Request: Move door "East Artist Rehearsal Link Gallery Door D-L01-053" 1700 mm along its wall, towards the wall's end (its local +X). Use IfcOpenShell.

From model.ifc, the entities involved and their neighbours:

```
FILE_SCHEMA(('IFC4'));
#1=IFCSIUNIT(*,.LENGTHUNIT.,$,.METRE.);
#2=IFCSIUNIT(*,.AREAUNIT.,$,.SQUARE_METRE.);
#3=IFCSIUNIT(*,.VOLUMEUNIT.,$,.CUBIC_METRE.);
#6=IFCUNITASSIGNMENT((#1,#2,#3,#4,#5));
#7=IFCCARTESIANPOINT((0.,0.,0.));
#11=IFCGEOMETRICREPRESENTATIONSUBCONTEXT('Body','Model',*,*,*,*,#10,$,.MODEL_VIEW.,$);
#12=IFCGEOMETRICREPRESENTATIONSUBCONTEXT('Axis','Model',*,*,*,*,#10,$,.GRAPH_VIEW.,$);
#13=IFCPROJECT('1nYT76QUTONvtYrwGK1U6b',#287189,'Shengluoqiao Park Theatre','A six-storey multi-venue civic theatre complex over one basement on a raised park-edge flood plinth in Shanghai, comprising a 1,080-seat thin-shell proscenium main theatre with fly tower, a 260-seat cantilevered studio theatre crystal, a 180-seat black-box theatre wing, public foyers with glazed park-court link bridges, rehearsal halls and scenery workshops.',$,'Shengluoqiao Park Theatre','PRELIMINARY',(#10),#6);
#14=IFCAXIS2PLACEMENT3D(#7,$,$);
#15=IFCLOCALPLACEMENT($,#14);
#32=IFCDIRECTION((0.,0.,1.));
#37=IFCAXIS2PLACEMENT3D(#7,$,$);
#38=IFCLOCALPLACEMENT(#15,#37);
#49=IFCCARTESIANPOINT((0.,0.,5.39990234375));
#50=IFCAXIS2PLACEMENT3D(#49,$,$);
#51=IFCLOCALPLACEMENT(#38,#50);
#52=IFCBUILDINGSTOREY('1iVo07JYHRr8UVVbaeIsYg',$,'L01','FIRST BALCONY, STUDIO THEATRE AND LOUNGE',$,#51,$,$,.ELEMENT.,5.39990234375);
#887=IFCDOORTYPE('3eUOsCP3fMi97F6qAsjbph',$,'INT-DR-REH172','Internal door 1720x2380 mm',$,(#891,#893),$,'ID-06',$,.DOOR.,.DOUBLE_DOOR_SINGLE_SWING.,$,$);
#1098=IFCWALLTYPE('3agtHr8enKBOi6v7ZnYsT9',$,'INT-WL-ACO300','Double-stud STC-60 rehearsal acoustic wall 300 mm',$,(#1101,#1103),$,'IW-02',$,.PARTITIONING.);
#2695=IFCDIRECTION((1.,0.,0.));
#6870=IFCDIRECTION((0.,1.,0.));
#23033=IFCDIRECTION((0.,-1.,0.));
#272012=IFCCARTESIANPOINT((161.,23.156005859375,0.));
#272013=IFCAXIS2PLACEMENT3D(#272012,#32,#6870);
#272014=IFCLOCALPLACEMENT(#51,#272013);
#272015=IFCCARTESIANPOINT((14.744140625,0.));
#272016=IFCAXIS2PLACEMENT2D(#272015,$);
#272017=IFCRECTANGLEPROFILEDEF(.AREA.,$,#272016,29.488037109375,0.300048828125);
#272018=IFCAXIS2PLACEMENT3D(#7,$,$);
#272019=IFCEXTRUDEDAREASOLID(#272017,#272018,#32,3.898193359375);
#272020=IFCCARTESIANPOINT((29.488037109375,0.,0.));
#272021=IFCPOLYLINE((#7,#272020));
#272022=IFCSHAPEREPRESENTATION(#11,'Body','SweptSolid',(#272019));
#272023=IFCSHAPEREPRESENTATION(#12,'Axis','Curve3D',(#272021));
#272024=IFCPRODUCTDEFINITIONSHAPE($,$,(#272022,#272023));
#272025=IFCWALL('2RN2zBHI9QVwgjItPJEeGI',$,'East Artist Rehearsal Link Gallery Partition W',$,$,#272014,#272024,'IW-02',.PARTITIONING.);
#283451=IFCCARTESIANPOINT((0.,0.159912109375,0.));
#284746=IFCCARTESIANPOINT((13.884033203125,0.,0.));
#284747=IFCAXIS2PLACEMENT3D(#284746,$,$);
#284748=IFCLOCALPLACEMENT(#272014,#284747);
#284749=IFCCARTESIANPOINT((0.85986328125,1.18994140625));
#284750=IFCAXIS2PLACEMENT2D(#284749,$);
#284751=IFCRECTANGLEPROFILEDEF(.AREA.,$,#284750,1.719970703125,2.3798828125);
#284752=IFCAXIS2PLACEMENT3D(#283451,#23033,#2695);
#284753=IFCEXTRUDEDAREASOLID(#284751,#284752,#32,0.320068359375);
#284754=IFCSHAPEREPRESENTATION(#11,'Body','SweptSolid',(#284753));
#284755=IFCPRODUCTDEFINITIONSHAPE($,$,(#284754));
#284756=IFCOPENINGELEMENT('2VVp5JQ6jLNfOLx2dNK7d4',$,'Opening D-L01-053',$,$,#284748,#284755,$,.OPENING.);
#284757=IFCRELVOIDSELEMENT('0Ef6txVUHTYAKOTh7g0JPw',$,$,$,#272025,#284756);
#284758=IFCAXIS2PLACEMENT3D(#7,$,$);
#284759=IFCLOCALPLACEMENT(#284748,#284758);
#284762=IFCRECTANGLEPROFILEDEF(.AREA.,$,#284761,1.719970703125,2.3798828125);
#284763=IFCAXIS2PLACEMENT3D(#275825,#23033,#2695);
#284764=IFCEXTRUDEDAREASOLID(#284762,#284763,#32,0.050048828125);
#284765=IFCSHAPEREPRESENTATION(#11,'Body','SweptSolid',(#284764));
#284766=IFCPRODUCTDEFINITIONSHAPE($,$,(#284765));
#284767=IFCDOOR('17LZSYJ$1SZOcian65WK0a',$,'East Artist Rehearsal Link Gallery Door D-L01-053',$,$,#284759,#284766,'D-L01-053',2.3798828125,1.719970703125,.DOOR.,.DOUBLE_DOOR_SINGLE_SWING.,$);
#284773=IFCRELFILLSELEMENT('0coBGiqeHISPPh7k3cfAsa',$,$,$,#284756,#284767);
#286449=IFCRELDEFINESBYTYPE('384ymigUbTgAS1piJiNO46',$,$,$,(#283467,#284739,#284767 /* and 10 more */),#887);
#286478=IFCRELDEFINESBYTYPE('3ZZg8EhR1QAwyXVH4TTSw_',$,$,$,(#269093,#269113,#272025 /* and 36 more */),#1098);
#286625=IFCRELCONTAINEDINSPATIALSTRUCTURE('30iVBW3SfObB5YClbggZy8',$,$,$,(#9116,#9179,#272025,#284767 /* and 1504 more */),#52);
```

```python
import ifcopenshell
import ifcopenshell.api.geometry
import ifcopenshell.util.placement

model = ifcopenshell.open("model.ifc")

door = model.by_id(284767)
opening = door.FillsVoids[0].RelatingOpeningElement
wall = opening.VoidsElements[0].RelatingBuildingElement

wall_matrix = ifcopenshell.util.placement.get_local_placement(wall.ObjectPlacement)
shift = wall_matrix[:3, 0] * 1.7
before = ifcopenshell.util.placement.get_local_placement(door.ObjectPlacement)[:3, 3].copy()

# The door is placed relative to its opening, so it follows when the opening moves.
matrix = ifcopenshell.util.placement.get_local_placement(opening.ObjectPlacement)
matrix[:3, 3] += shift
ifcopenshell.api.geometry.edit_object_placement(
    model, product=opening, matrix=matrix, is_si=False, should_transform_children=True
)

after = ifcopenshell.util.placement.get_local_placement(door.ObjectPlacement)[:3, 3]
print("door moved by", (after - before).round(3) + 0.0)

model.write("model_edited.ifc")
```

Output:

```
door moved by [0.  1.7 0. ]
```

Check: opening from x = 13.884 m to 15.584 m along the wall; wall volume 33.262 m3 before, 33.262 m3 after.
